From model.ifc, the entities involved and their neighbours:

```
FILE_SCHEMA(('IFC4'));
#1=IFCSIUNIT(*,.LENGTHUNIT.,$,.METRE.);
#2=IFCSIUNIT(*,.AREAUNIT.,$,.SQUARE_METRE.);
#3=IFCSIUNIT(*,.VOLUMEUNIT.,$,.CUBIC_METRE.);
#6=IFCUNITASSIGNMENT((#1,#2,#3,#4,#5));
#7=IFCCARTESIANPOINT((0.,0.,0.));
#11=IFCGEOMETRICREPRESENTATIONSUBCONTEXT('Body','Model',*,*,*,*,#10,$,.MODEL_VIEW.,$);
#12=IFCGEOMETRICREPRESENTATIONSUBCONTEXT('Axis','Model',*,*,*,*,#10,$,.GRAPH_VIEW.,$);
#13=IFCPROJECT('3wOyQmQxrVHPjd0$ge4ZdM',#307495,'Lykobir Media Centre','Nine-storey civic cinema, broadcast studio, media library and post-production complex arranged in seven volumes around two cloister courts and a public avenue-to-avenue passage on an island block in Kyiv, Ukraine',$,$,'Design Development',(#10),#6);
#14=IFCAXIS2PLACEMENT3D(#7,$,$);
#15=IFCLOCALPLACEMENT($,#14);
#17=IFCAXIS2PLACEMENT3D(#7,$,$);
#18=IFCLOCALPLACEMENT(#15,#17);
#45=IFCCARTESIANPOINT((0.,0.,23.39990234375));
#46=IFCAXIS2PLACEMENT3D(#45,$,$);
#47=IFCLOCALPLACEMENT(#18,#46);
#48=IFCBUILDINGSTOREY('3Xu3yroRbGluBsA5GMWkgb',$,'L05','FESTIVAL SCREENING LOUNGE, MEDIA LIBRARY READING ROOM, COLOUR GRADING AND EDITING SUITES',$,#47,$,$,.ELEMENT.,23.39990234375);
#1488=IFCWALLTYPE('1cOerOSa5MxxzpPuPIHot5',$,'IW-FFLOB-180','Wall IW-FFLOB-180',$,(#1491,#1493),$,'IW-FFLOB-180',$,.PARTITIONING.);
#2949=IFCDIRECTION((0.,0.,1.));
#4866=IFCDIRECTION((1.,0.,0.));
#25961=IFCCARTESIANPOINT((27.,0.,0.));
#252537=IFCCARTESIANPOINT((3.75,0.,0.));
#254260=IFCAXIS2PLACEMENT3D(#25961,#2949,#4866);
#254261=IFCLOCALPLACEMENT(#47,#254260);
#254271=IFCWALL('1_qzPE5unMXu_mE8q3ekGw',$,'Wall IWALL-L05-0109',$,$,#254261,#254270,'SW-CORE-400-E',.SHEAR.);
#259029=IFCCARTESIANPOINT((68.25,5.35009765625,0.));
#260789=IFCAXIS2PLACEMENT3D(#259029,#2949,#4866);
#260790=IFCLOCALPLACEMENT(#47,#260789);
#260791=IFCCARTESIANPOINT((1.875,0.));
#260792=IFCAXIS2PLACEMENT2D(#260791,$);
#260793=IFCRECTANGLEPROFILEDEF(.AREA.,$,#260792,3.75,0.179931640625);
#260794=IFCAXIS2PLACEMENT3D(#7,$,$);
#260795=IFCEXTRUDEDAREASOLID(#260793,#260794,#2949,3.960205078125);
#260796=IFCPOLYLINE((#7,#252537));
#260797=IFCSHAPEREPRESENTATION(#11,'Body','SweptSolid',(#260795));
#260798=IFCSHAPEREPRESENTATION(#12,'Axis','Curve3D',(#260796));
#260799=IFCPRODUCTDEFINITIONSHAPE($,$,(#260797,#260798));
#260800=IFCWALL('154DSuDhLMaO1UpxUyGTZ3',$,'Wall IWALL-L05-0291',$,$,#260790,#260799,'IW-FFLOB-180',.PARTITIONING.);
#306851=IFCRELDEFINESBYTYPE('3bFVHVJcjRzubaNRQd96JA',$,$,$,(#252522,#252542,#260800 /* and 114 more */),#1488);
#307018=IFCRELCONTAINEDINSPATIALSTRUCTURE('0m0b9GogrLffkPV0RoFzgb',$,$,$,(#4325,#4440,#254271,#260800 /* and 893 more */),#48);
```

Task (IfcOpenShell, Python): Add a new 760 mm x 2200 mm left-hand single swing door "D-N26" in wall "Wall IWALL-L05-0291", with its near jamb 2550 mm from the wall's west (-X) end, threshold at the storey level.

```python
import numpy as np
import ifcopenshell
import ifcopenshell.api.feature
import ifcopenshell.api.geometry
import ifcopenshell.api.root
import ifcopenshell.api.spatial
import ifcopenshell.geom
import ifcopenshell.util.element
import ifcopenshell.util.placement
import ifcopenshell.util.representation
import ifcopenshell.util.shape
import ifcopenshell.util.unit

model = ifcopenshell.open("model.ifc")
unit_scale = ifcopenshell.util.unit.calculate_unit_scale(model)
settings = ifcopenshell.geom.settings()


def volume(element):
    """Net volume in cubic metres, openings subtracted."""
    shape = ifcopenshell.geom.create_shape(settings, element)
    return ifcopenshell.util.shape.get_volume(shape.geometry)


wall = model.by_guid("154DSuDhLMaO1UpxUyGTZ3")
storey = ifcopenshell.util.element.get_container(wall, ifc_class="IfcBuildingStorey")
context = ifcopenshell.util.representation.get_context(model, "Model", "Body", "MODEL_VIEW")
before = volume(wall)

width, height, from_end, sill = 0.76, 2.2, 2.55, 0.0  # metres

# The wall runs along its own X axis, and the end named is its -X end.
wall_shape = ifcopenshell.geom.create_shape(settings, wall)
x, y, z = ifcopenshell.util.shape.get_vertices(wall_shape.geometry).T
start = x.min() + from_end
face, thickness = float(y.min()), float(y.max() - y.min())
wall_matrix = ifcopenshell.util.placement.get_local_placement(wall.ObjectPlacement)
level = ifcopenshell.util.placement.get_local_placement(storey.ObjectPlacement)[2, 3]


def in_wall(x, y):
    """Placement at x, y metres in the wall's axes, at sill height."""
    matrix = wall_matrix.copy()
    matrix[:, 3] = wall_matrix @ np.array([x / unit_scale, y / unit_scale, 0.0, 1.0])
    matrix[2, 3] = level + sill / unit_scale
    return matrix


# Opening: a box that overshoots both wall faces by 50 mm.
opening = ifcopenshell.api.root.create_entity(model, ifc_class="IfcOpeningElement", predefined_type="OPENING")
box = ifcopenshell.api.geometry.add_wall_representation(
    model, context=context, length=width, height=height, thickness=thickness + 0.1
)
ifcopenshell.api.geometry.assign_representation(model, product=opening, representation=box)
ifcopenshell.api.geometry.edit_object_placement(model, product=opening, matrix=in_wall(start, face - 0.05), is_si=False)
ifcopenshell.api.feature.add_feature(model, feature=opening, element=wall)

door = ifcopenshell.api.root.create_entity(model, ifc_class="IfcDoor", name="D-N26", predefined_type="DOOR")
door.OverallWidth, door.OverallHeight = width / unit_scale, height / unit_scale
door.OperationType = "SINGLE_SWING_LEFT"
body = ifcopenshell.api.geometry.add_door_representation(
    model,
    context=context,
    overall_width=door.OverallWidth,
    overall_height=door.OverallHeight,
    operation_type="SINGLE_SWING_LEFT",
    lining_properties={"LiningDepth": thickness / unit_scale, "ThresholdDepth": thickness / unit_scale},
)
ifcopenshell.api.geometry.assign_representation(model, product=door, representation=body)
ifcopenshell.api.spatial.assign_container(model, products=[door], relating_structure=storey)
ifcopenshell.api.feature.add_filling(model, opening=opening, element=door)

# The lining spans the wall, so the door starts at the wall face.
ifcopenshell.api.geometry.edit_object_placement(model, product=door, matrix=in_wall(start, face), is_si=False)

after = volume(wall)

print(f"wall volume {before:.3f} -> {after:.3f} m3")

model.write("model_updated.ifc")
```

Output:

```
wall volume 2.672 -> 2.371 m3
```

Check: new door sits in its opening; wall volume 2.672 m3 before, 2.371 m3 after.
